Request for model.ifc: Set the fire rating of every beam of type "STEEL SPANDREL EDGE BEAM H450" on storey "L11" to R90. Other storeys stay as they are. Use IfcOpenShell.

First a look at what the model holds.

```python
import ifcopenshell
import ifcopenshell.util.element

model = ifcopenshell.open("model.ifc")
print(model.schema)
storey = next(s for s in model.by_type("IfcBuildingStorey") if s.Name == "L11")
beams = [e for e in ifcopenshell.util.element.get_decomposition(storey) if e.is_a("IfcBeam")]
seen = {}
for e in beams:
    element_type = ifcopenshell.util.element.get_type(e)
    key = (element_type.Name if element_type != e and element_type else None, ifcopenshell.util.element.get_pset(e, "Pset_BeamCommon", "FireRating"))
    seen[key] = seen.get(key, 0) + 1
for (name, value), count in sorted(seen.items(), key=str):
    print(count, "x", name, "|", value)
```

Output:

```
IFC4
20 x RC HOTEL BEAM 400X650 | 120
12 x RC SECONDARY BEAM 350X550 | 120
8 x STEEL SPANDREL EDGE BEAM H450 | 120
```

```python
import ifcopenshell
import ifcopenshell.api.pset
import ifcopenshell.util.element

model = ifcopenshell.open("model.ifc")

storey = next(s for s in model.by_type("IfcBuildingStorey") if s.Name == "L11")
beams = [e for e in ifcopenshell.util.element.get_decomposition(storey) if e.is_a("IfcBeam")]

count = 0
for e in beams:
    element_type = ifcopenshell.util.element.get_type(e)
    if element_type in (None, e) or element_type.Name != "STEEL SPANDREL EDGE BEAM H450":
        continue
    # add_pset returns the element's existing set when there is one.
    pset = ifcopenshell.api.pset.add_pset(model, product=e, name="Pset_BeamCommon")
    ifcopenshell.api.pset.edit_pset(model, pset=pset, properties={"FireRating": "R90"})
    count += 1

print(count, "beams updated")

model.write("model_rev.ifc")
```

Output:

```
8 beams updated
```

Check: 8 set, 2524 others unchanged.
